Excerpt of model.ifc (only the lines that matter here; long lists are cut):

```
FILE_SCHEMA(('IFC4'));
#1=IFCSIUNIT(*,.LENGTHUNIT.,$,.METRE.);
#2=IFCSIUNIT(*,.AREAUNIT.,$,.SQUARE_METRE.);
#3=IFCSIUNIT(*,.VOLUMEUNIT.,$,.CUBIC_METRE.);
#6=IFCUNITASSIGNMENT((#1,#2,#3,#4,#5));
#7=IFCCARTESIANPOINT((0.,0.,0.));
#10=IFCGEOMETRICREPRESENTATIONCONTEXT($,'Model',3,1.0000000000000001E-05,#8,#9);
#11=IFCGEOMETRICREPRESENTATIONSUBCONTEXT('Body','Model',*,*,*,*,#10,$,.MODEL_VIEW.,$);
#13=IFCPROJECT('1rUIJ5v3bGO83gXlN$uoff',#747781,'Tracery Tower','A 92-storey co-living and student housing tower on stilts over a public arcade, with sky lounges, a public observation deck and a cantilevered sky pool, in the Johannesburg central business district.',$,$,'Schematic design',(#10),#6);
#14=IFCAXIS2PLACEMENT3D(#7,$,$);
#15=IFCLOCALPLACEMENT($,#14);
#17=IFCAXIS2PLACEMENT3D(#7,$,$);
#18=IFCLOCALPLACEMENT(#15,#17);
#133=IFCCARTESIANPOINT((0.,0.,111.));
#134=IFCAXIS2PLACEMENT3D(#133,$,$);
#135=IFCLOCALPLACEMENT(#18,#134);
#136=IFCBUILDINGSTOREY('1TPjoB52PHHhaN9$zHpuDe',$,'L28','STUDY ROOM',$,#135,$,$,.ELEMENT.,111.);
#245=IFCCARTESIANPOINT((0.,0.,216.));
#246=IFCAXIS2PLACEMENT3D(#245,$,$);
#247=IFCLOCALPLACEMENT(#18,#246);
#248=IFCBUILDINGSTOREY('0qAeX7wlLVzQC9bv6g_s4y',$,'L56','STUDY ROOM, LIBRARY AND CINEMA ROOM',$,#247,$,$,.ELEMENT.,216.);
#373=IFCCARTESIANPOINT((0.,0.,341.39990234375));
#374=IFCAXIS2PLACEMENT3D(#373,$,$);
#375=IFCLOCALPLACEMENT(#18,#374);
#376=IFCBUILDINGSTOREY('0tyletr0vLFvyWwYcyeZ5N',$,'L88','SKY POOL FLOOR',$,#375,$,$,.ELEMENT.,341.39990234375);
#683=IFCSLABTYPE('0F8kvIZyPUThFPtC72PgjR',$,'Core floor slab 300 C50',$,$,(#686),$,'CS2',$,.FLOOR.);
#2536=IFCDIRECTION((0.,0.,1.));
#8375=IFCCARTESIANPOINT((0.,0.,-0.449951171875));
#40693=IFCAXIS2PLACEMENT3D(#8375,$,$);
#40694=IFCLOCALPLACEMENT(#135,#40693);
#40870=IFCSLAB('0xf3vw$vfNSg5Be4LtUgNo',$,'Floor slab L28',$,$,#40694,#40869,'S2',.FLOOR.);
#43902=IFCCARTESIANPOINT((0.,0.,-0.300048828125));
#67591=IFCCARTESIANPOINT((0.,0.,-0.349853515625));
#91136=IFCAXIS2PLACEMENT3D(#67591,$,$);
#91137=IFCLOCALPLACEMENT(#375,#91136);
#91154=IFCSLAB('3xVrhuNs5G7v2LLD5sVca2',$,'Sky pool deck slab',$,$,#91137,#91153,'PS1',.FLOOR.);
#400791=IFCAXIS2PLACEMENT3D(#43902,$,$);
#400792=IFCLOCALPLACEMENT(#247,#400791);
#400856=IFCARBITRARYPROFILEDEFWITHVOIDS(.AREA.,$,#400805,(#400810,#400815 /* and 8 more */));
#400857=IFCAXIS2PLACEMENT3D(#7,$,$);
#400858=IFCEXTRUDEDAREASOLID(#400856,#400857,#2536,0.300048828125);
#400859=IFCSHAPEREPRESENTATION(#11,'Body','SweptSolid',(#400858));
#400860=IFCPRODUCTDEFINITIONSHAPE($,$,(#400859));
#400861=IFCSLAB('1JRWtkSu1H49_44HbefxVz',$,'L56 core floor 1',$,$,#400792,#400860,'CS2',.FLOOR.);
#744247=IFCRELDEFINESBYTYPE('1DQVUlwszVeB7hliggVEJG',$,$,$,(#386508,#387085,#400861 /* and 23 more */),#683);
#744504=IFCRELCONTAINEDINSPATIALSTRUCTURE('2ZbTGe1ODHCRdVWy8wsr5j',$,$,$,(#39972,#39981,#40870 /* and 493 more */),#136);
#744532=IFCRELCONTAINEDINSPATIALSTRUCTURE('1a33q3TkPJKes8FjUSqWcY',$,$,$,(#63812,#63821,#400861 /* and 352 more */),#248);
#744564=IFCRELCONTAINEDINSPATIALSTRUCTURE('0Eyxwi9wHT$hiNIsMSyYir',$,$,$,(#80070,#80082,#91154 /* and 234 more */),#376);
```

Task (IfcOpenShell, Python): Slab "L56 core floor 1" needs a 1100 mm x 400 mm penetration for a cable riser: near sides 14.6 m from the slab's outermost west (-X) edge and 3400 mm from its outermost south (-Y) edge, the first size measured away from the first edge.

```python
import numpy as np
import ifcopenshell
import ifcopenshell.api.feature
import ifcopenshell.api.geometry
import ifcopenshell.api.root
import ifcopenshell.geom
import ifcopenshell.util.placement
import ifcopenshell.util.representation
import ifcopenshell.util.shape
import ifcopenshell.util.unit

model = ifcopenshell.open("model.ifc")
unit_scale = ifcopenshell.util.unit.calculate_unit_scale(model)
settings = ifcopenshell.geom.settings()


def volume(element):
    """Net volume in cubic metres, openings subtracted."""
    shape = ifcopenshell.geom.create_shape(settings, element)
    return ifcopenshell.util.shape.get_volume(shape.geometry)


slab = model.by_id(400861)
before = volume(slab)

# Extent in the slab's own axes, in metres. The edges named are its -X and -Y sides.
slab_shape = ifcopenshell.geom.create_shape(settings, slab)
vertices = ifcopenshell.util.shape.get_vertices(slab_shape.geometry)
x_min, y_min, bottom = vertices.min(axis=0)
top = vertices[:, 2].max()

opening = ifcopenshell.api.root.create_entity(model, ifc_class="IfcOpeningElement", name="Cable riser opening", predefined_type="OPENING")
context = ifcopenshell.util.representation.get_context(model, "Model", "Body", "MODEL_VIEW")
width, depth = 1.1, 0.4
outline = [(0.0, 0.0), (width, 0.0), (width, depth), (0.0, depth), (0.0, 0.0)]
# Overshoot both faces by 50 mm so the cut is clean.
shape = ifcopenshell.api.geometry.add_slab_representation(
    model, context=context, depth=top - bottom + 0.1, polyline=outline
)
ifcopenshell.api.geometry.assign_representation(model, product=opening, representation=shape)

matrix = ifcopenshell.util.placement.get_local_placement(slab.ObjectPlacement)
matrix[:, 3] = matrix @ np.append(np.array([x_min + 14.6, y_min + 3.4, bottom - 0.05]) / unit_scale, 1.0)
ifcopenshell.api.geometry.edit_object_placement(model, product=opening, matrix=matrix, is_si=False)
ifcopenshell.api.feature.add_feature(model, feature=opening, element=slab)

after = volume(slab)

print(f"slab volume {before:.3f} -> {after:.3f} m3")

model.write("model_v2.ifc")
```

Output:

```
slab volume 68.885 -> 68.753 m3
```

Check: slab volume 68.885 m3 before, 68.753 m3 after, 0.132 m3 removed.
